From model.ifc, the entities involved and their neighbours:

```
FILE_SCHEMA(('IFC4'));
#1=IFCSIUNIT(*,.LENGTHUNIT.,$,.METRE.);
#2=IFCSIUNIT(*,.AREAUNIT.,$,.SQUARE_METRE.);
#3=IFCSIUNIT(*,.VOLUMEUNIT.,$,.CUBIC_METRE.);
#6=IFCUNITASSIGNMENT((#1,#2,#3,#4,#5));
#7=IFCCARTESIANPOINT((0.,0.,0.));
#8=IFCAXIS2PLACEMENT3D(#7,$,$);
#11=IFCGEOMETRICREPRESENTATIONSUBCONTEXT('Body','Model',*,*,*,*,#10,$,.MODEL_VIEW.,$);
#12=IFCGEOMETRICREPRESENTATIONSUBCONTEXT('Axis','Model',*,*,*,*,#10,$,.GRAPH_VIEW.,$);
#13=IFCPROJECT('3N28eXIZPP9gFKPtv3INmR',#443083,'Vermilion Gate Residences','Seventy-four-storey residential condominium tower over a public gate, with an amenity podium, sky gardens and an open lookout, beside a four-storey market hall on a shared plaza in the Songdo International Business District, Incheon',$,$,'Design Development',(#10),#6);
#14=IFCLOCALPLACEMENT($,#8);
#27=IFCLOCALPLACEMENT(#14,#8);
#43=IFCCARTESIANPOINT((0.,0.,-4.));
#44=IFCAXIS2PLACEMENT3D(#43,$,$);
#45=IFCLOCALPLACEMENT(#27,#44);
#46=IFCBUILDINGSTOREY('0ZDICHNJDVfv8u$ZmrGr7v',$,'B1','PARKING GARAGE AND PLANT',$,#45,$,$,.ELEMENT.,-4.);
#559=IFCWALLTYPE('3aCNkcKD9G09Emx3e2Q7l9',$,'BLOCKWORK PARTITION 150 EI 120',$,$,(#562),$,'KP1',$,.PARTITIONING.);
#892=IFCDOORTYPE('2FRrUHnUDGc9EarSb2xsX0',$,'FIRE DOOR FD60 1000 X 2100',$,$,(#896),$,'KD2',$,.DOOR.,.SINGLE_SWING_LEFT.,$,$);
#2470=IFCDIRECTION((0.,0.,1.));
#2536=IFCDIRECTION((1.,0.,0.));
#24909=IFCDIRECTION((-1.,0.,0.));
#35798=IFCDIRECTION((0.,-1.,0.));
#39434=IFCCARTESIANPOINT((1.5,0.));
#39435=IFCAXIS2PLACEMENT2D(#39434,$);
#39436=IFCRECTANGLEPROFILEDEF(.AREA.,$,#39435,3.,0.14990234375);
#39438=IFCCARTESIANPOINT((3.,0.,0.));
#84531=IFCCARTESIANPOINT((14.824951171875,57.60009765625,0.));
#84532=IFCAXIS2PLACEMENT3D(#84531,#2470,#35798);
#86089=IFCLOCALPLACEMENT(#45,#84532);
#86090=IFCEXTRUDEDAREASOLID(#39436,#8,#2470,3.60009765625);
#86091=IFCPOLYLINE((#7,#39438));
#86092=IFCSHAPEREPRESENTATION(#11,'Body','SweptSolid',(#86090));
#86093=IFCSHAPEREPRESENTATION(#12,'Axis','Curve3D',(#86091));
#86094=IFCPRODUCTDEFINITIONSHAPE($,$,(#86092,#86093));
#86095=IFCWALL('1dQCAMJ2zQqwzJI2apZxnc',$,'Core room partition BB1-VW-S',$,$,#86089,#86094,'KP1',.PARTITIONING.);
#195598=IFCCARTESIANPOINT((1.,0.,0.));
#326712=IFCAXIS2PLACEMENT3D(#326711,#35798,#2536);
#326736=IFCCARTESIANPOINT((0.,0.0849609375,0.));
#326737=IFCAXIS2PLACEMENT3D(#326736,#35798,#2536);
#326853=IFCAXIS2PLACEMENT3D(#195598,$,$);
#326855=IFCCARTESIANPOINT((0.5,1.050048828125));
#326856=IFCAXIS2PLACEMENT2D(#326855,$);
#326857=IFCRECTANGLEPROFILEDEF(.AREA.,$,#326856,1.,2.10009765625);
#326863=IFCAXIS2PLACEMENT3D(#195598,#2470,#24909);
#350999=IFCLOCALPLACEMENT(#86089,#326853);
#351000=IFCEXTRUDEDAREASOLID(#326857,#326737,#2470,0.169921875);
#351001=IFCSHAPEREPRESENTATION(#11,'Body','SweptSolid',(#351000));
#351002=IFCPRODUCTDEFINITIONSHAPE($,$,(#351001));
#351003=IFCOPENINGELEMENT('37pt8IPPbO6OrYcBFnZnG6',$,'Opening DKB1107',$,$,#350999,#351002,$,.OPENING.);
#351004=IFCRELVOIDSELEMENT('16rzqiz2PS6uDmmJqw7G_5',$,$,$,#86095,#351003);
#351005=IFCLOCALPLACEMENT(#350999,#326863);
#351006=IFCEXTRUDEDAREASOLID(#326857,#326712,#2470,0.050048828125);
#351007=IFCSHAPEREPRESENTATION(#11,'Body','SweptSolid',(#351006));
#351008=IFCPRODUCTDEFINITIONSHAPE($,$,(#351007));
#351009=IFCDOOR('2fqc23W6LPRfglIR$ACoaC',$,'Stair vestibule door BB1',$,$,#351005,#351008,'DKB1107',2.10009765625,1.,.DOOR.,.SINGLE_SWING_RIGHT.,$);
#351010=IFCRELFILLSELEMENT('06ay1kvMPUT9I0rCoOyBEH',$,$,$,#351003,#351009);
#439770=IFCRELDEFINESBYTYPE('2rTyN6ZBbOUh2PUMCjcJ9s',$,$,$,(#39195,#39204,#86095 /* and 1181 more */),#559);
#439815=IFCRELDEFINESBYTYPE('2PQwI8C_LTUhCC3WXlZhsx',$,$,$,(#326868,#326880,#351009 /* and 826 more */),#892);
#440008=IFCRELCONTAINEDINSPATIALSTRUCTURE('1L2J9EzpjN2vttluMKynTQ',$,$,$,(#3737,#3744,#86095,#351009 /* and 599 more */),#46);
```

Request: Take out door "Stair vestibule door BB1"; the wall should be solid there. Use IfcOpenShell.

```python
import ifcopenshell
import ifcopenshell.api.feature
import ifcopenshell.api.root
import ifcopenshell.geom
import ifcopenshell.util.shape

model = ifcopenshell.open("model.ifc")
settings = ifcopenshell.geom.settings()


def volume(element):
    """Net volume in cubic metres, openings subtracted."""
    shape = ifcopenshell.geom.create_shape(settings, element)
    return ifcopenshell.util.shape.get_volume(shape.geometry)


door = model.by_guid("2fqc23W6LPRfglIR$ACoaC")
opening = door.FillsVoids[0].RelatingOpeningElement
wall = opening.VoidsElements[0].RelatingBuildingElement
before = volume(wall)

ifcopenshell.api.root.remove_product(model, product=door)
ifcopenshell.api.feature.remove_feature(model, feature=opening)

after = volume(wall)

print(f"wall volume {before:.3f} -> {after:.3f} m3")

model.write("model-out.ifc")
```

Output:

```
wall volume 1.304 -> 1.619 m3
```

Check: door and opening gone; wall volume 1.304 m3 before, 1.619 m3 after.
